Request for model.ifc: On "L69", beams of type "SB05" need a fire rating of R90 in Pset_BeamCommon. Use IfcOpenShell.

First a look at what the model holds.

```python
import ifcopenshell
import ifcopenshell.util.element

model = ifcopenshell.open("model.ifc")
print(model.schema)
storey = next(s for s in model.by_type("IfcBuildingStorey") if s.Name == "L69")
beams = [e for e in ifcopenshell.util.element.get_decomposition(storey) if e.is_a("IfcBeam")]
seen = {}
for e in beams:
    element_type = ifcopenshell.util.element.get_type(e)
    key = (element_type.Name if element_type != e and element_type else None, ifcopenshell.util.element.get_pset(e, "Pset_BeamCommon", "FireRating"))
    seen[key] = seen.get(key, 0) + 1
for (name, value), count in sorted(seen.items(), key=str):
    print(count, "x", name, "|", value)
```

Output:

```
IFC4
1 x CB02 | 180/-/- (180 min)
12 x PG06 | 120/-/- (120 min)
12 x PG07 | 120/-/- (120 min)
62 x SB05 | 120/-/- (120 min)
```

```python
import ifcopenshell
import ifcopenshell.api.pset
import ifcopenshell.util.element

model = ifcopenshell.open("model.ifc")

storey = next(s for s in model.by_type("IfcBuildingStorey") if s.Name == "L69")
beams = [e for e in ifcopenshell.util.element.get_decomposition(storey) if e.is_a("IfcBeam")]

count = 0
for e in beams:
    element_type = ifcopenshell.util.element.get_type(e)
    if element_type in (None, e) or element_type.Name != "SB05":
        continue
    found = ifcopenshell.util.element.get_pset(e, "Pset_BeamCommon", should_inherit=False)
    if found:
        pset = model.by_id(found["id"])
        if len(ifcopenshell.util.element.get_elements_by_pset(pset)) > 1:
            pset = ifcopenshell.api.pset.unshare_pset(model, products=[e], pset=pset)[0]
    else:
        pset = ifcopenshell.api.pset.add_pset(model, product=e, name="Pset_BeamCommon")
    ifcopenshell.api.pset.edit_pset(model, pset=pset, properties={"FireRating": "R90"})
    count += 1

print(count, "beams updated")

model.write("model_rev.ifc")
```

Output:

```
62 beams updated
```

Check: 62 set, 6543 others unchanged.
